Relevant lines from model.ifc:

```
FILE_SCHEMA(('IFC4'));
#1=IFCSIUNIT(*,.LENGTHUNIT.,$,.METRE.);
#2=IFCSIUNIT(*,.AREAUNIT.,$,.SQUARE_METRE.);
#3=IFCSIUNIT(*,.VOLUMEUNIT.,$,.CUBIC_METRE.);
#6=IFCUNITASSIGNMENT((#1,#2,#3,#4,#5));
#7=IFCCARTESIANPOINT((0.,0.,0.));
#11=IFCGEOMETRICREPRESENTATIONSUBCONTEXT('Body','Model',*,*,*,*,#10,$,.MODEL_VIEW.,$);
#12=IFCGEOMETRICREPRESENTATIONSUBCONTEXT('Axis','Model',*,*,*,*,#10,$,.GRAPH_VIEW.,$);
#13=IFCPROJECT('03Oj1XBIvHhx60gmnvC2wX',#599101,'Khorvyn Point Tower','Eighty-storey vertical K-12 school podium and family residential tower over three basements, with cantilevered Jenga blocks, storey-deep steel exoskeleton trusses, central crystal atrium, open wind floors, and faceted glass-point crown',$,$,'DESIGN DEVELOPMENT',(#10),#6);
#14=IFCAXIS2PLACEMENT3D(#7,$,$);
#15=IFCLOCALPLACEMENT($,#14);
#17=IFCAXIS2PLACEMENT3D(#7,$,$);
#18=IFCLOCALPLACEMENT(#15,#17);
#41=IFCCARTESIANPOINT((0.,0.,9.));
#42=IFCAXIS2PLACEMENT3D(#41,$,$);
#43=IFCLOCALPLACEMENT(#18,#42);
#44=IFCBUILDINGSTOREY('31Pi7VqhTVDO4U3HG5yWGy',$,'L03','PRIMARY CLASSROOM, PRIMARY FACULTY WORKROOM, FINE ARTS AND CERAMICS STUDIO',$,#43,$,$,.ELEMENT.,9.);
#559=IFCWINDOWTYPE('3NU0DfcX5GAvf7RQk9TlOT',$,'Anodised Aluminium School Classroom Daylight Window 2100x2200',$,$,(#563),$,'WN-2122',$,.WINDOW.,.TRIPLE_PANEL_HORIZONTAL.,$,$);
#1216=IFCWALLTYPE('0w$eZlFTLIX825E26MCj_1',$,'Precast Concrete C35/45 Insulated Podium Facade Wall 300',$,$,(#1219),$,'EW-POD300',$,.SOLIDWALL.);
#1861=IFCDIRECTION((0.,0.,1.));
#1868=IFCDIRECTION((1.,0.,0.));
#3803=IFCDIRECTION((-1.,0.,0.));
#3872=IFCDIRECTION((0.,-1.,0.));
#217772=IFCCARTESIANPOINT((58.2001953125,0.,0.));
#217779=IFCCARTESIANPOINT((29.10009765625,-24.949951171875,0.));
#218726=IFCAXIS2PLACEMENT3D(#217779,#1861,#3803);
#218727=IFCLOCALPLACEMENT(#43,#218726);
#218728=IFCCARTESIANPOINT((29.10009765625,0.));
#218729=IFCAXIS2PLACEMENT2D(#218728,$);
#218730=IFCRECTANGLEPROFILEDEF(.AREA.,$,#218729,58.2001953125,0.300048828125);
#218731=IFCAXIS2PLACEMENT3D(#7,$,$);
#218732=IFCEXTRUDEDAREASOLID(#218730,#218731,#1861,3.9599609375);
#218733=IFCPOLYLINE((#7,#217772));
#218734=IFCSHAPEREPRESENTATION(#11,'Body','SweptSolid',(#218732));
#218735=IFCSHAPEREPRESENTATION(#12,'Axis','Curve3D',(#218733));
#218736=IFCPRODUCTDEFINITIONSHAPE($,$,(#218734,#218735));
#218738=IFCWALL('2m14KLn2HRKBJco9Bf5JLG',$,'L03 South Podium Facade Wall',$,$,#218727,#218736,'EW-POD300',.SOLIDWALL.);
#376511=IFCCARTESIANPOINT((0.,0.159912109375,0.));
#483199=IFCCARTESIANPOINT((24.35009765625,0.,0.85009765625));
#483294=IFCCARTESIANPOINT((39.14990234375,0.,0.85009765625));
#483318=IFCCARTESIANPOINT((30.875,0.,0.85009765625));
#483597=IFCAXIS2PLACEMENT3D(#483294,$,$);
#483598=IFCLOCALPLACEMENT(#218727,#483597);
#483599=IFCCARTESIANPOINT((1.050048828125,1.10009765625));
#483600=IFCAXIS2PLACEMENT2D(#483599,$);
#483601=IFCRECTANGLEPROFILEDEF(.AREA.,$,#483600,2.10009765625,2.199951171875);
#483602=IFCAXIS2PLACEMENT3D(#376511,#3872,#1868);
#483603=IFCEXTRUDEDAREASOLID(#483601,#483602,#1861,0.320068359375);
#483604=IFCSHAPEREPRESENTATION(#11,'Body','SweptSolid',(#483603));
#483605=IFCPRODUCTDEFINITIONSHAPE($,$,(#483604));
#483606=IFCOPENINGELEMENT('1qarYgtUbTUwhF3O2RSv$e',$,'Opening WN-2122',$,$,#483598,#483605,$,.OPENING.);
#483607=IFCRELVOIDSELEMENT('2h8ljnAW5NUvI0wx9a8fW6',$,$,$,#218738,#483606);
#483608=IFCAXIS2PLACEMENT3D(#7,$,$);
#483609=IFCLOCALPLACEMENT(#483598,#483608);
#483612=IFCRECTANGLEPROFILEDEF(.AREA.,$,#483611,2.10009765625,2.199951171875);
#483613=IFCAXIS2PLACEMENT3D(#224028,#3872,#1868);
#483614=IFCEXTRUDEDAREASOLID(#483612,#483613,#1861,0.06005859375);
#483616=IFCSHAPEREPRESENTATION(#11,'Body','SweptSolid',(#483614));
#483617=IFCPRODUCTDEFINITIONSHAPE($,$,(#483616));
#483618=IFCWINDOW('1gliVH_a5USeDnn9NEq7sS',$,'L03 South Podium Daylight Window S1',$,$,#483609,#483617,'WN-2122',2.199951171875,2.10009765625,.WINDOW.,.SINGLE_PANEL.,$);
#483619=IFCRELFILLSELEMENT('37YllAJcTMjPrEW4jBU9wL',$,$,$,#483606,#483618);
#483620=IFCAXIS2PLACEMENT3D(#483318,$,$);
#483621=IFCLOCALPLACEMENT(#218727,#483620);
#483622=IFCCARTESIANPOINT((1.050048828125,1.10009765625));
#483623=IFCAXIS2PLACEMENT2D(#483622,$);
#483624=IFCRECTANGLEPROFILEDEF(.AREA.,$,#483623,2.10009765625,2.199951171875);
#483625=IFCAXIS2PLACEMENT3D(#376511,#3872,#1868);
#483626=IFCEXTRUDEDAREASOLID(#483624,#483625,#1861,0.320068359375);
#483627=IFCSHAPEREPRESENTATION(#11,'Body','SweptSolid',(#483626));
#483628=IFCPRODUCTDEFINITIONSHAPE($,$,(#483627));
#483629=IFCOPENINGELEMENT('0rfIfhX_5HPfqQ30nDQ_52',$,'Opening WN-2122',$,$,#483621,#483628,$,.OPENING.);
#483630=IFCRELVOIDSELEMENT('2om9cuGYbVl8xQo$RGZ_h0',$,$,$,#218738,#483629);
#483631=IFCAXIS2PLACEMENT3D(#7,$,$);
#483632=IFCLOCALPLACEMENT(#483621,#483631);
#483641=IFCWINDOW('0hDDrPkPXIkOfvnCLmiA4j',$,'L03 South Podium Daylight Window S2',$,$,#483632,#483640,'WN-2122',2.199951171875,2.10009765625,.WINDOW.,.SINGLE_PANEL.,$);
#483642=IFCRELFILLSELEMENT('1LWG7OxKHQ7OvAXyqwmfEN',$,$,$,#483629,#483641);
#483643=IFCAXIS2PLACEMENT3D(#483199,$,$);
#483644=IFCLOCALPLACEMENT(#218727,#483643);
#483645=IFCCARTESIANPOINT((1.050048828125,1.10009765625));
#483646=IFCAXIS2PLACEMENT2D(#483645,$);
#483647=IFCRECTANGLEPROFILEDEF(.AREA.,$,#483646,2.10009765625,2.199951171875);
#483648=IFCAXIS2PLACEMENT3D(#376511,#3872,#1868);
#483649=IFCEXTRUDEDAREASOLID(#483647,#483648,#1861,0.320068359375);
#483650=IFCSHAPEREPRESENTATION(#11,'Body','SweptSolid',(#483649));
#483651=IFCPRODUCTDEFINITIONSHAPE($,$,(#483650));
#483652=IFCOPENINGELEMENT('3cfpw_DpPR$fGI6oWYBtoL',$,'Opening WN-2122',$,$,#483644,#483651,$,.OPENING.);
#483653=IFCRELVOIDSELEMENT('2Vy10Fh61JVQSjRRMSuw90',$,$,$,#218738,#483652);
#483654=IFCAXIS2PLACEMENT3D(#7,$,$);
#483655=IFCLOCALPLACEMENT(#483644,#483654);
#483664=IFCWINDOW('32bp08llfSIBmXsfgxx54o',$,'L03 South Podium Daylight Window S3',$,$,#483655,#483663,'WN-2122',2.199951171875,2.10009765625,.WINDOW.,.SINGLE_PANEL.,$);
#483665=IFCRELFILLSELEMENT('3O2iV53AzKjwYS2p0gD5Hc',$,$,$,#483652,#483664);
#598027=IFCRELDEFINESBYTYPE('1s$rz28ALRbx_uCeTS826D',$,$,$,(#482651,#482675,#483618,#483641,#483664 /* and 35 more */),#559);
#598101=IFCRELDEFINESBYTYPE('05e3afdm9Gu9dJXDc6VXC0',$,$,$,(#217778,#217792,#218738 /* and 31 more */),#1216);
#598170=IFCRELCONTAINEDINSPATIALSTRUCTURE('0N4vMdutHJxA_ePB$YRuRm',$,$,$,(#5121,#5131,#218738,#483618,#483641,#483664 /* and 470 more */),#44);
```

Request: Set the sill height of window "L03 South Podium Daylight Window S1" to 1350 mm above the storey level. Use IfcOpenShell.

```python
import numpy as np
import ifcopenshell
import ifcopenshell.api.geometry
import ifcopenshell.geom
import ifcopenshell.util.element
import ifcopenshell.util.placement
import ifcopenshell.util.shape
import ifcopenshell.util.unit

model = ifcopenshell.open("model.ifc")
unit_scale = ifcopenshell.util.unit.calculate_unit_scale(model)

window = model.by_guid("1gliVH_a5USeDnn9NEq7sS")
opening = window.FillsVoids[0].RelatingOpeningElement
storey = ifcopenshell.util.element.get_container(window, ifc_class="IfcBuildingStorey")
level = ifcopenshell.util.placement.get_local_placement(storey.ObjectPlacement)[2, 3]

# The opening's origin need not be at the sill, so measure its lowest point.
shape = ifcopenshell.geom.create_shape(ifcopenshell.geom.settings(), opening)
bottom = ifcopenshell.util.shape.get_shape_bottom_elevation(shape, shape.geometry) / unit_scale
dz = level + 1.35 - bottom

shift = np.array([0.0, 0.0, dz])
# The window is placed relative to its opening, so it follows when the opening moves.
matrix = ifcopenshell.util.placement.get_local_placement(opening.ObjectPlacement)
matrix[:3, 3] += shift
ifcopenshell.api.geometry.edit_object_placement(
    model, product=opening, matrix=matrix, is_si=False, should_transform_children=True
)

print(f"moved by {dz * unit_scale:+.3f} m")

model.write("model_edited.ifc")
```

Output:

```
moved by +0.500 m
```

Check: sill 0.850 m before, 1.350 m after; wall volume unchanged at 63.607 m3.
